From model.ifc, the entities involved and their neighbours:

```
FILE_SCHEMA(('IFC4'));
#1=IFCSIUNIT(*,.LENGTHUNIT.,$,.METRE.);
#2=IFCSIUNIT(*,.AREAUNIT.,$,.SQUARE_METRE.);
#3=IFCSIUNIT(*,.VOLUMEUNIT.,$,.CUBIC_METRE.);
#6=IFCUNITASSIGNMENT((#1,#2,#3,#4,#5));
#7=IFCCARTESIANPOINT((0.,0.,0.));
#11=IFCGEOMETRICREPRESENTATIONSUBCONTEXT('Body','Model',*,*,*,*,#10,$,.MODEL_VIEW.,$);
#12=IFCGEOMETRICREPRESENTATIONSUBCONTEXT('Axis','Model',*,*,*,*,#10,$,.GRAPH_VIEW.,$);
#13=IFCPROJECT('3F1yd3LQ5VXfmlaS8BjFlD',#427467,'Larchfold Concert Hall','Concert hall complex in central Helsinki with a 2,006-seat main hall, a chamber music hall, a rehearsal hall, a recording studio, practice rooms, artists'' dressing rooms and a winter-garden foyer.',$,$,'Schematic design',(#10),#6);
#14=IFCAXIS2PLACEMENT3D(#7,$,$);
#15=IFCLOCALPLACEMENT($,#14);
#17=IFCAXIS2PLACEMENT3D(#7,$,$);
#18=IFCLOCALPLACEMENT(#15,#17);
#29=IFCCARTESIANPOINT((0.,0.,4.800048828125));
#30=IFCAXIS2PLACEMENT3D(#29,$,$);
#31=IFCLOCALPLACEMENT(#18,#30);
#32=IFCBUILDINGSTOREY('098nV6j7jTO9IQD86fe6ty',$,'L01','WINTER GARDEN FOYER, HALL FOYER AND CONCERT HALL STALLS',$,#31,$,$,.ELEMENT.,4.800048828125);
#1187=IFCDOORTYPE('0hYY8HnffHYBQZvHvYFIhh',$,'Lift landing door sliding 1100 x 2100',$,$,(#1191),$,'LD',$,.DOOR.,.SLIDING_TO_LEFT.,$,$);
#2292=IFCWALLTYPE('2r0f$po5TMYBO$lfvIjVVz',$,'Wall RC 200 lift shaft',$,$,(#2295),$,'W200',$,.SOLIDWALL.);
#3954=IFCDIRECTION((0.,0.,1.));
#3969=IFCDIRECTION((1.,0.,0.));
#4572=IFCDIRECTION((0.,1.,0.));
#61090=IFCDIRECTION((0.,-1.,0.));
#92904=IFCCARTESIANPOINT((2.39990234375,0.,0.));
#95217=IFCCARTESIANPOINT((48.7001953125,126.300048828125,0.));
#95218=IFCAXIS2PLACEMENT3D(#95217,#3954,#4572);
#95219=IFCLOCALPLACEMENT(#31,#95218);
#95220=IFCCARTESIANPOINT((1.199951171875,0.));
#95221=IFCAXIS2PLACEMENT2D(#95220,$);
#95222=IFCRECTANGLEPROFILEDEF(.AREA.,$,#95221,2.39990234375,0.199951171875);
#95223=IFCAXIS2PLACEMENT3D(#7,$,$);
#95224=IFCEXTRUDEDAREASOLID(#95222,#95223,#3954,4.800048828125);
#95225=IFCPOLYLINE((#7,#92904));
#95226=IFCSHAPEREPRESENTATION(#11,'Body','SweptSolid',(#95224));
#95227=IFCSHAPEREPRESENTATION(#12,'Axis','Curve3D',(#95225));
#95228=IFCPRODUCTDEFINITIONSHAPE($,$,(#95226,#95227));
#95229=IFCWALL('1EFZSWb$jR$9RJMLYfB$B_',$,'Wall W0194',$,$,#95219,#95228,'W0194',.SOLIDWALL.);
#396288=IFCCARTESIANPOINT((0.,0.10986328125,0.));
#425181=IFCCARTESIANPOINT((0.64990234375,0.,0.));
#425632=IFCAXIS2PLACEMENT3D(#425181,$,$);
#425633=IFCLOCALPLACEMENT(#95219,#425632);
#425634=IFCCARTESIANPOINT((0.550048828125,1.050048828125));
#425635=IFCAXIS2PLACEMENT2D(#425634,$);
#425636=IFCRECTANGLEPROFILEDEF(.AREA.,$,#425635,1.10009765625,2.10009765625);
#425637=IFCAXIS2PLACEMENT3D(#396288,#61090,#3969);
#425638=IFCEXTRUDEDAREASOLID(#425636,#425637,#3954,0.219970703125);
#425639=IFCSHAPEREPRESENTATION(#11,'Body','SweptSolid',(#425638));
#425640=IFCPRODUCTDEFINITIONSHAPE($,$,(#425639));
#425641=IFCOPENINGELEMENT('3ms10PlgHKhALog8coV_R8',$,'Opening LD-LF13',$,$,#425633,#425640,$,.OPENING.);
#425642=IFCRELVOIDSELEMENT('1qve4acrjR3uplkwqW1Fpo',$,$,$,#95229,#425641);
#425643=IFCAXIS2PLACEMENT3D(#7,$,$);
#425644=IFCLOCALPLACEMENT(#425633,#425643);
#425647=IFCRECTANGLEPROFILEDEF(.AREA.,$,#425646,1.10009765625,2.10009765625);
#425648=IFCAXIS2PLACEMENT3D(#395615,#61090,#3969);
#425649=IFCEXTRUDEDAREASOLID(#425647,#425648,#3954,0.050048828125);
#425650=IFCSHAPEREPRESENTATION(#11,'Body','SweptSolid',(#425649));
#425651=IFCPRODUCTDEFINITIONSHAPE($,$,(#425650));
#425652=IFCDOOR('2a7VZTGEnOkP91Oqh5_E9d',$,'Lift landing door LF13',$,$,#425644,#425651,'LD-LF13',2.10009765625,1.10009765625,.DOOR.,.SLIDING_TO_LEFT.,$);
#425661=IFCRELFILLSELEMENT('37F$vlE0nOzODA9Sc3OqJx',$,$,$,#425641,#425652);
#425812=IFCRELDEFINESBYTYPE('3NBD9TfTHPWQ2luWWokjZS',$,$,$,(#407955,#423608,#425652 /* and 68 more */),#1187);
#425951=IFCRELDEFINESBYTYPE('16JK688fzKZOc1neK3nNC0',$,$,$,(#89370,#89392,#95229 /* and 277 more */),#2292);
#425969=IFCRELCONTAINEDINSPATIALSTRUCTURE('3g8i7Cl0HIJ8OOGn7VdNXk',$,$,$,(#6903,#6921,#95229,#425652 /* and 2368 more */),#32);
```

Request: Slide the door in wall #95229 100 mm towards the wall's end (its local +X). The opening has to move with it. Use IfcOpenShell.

```python
import ifcopenshell
import ifcopenshell.api.geometry
import ifcopenshell.util.placement
import ifcopenshell.util.unit

model = ifcopenshell.open("model.ifc")
unit_scale = ifcopenshell.util.unit.calculate_unit_scale(model)

door = model.by_guid("2a7VZTGEnOkP91Oqh5_E9d")
opening = door.FillsVoids[0].RelatingOpeningElement
wall = opening.VoidsElements[0].RelatingBuildingElement

wall_matrix = ifcopenshell.util.placement.get_local_placement(wall.ObjectPlacement)
shift = wall_matrix[:3, 0] * 0.1 / unit_scale
before = ifcopenshell.util.placement.get_local_placement(door.ObjectPlacement)[:3, 3].copy()

# The door is placed relative to its opening, so it follows when the opening moves.
matrix = ifcopenshell.util.placement.get_local_placement(opening.ObjectPlacement)
matrix[:3, 3] += shift
ifcopenshell.api.geometry.edit_object_placement(
    model, product=opening, matrix=matrix, is_si=False, should_transform_children=True
)

after = ifcopenshell.util.placement.get_local_placement(door.ObjectPlacement)[:3, 3]
print("door moved by", (after - before).round(3) + 0.0)

model.write("model_updated.ifc")
```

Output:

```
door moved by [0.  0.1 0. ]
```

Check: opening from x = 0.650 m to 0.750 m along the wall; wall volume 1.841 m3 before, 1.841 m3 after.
